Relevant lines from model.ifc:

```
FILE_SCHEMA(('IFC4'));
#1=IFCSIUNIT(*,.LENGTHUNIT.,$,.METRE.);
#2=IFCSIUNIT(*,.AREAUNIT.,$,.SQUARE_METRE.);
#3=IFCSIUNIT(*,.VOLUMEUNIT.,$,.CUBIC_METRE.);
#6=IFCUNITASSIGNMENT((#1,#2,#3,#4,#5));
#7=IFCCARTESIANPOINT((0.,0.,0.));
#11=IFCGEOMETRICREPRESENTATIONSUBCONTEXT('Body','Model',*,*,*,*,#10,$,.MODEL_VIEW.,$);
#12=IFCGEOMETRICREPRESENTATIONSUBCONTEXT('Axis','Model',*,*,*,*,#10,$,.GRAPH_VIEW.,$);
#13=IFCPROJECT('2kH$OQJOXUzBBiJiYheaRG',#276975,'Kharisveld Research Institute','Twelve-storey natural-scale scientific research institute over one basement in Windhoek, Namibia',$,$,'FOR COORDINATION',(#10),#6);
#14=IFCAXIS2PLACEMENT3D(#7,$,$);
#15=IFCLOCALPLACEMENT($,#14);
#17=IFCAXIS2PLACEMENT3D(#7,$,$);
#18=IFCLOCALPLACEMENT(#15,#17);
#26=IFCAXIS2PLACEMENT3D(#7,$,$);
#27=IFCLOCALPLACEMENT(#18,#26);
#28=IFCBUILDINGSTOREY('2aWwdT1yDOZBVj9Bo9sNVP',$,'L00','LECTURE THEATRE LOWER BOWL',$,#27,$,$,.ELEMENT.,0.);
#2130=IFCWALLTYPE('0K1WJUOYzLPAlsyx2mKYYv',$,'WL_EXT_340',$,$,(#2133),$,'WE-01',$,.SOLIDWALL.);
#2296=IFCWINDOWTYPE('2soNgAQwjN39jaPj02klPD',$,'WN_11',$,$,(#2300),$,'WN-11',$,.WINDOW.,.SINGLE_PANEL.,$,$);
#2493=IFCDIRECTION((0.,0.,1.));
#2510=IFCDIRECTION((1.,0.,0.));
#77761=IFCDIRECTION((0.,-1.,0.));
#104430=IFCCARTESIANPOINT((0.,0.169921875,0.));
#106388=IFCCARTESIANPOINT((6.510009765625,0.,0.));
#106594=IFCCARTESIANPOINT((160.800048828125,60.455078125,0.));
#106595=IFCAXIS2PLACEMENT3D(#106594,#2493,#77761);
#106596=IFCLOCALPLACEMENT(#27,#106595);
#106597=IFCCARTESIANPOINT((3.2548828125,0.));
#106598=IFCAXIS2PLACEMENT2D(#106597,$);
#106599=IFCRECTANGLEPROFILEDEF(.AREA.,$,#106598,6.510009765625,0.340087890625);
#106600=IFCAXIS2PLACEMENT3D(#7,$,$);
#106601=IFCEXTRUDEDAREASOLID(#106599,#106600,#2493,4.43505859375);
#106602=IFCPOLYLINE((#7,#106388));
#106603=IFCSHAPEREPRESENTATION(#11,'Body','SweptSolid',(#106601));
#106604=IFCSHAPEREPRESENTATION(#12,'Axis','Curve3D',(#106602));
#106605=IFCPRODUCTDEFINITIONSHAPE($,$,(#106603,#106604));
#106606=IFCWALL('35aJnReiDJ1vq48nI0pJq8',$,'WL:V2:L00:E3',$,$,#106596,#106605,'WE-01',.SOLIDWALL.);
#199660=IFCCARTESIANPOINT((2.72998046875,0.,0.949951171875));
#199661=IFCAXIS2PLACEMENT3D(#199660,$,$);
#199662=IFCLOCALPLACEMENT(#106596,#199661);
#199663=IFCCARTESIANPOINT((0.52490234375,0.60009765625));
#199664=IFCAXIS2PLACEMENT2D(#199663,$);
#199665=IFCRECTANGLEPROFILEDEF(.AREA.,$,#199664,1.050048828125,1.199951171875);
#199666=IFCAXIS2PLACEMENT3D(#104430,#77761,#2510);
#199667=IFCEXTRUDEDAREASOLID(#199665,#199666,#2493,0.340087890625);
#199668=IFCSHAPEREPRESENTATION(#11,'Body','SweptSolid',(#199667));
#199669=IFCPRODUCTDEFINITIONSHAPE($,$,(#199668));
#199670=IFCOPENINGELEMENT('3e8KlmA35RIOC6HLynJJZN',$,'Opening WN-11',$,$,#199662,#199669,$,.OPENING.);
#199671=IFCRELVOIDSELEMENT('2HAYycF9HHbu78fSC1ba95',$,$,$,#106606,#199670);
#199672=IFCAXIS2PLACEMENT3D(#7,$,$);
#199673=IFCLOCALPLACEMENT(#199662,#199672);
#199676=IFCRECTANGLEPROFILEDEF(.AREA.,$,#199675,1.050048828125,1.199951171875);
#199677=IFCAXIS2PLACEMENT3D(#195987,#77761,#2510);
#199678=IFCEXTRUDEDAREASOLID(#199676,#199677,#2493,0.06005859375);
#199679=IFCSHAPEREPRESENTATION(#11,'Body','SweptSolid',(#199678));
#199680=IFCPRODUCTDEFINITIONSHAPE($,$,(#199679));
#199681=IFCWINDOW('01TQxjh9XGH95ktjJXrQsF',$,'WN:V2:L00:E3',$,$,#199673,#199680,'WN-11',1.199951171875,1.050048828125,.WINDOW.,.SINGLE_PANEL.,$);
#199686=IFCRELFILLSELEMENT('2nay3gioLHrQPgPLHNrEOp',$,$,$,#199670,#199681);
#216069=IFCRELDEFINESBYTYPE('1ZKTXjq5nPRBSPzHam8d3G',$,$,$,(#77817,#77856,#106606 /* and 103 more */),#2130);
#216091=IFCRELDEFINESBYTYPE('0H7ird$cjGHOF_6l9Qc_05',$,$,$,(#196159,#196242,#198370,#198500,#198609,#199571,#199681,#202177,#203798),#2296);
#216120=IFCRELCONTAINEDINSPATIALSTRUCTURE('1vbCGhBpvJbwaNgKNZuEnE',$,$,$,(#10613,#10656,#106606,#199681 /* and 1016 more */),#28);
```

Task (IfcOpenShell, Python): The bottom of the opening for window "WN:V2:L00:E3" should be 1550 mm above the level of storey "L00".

```python
import numpy as np
import ifcopenshell
import ifcopenshell.api.geometry
import ifcopenshell.geom
import ifcopenshell.util.element
import ifcopenshell.util.placement
import ifcopenshell.util.shape
import ifcopenshell.util.unit

model = ifcopenshell.open("model.ifc")
unit_scale = ifcopenshell.util.unit.calculate_unit_scale(model)

window = model.by_guid("01TQxjh9XGH95ktjJXrQsF")
opening = window.FillsVoids[0].RelatingOpeningElement
storey = ifcopenshell.util.element.get_container(window, ifc_class="IfcBuildingStorey")
level = ifcopenshell.util.placement.get_local_placement(storey.ObjectPlacement)[2, 3]

# The opening's origin need not be at the sill, so measure its lowest point.
shape = ifcopenshell.geom.create_shape(ifcopenshell.geom.settings(), opening)
bottom = ifcopenshell.util.shape.get_shape_bottom_elevation(shape, shape.geometry) / unit_scale
dz = level + 1.55 - bottom

shift = np.array([0.0, 0.0, dz])
# The window is placed relative to its opening, so it follows when the opening moves.
matrix = ifcopenshell.util.placement.get_local_placement(opening.ObjectPlacement)
matrix[:3, 3] += shift
ifcopenshell.api.geometry.edit_object_placement(
    model, product=opening, matrix=matrix, is_si=False, should_transform_children=True
)

print(f"moved by {dz * unit_scale:+.3f} m")

model.write("model_edited.ifc")
```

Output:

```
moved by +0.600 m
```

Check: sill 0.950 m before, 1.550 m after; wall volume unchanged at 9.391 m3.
